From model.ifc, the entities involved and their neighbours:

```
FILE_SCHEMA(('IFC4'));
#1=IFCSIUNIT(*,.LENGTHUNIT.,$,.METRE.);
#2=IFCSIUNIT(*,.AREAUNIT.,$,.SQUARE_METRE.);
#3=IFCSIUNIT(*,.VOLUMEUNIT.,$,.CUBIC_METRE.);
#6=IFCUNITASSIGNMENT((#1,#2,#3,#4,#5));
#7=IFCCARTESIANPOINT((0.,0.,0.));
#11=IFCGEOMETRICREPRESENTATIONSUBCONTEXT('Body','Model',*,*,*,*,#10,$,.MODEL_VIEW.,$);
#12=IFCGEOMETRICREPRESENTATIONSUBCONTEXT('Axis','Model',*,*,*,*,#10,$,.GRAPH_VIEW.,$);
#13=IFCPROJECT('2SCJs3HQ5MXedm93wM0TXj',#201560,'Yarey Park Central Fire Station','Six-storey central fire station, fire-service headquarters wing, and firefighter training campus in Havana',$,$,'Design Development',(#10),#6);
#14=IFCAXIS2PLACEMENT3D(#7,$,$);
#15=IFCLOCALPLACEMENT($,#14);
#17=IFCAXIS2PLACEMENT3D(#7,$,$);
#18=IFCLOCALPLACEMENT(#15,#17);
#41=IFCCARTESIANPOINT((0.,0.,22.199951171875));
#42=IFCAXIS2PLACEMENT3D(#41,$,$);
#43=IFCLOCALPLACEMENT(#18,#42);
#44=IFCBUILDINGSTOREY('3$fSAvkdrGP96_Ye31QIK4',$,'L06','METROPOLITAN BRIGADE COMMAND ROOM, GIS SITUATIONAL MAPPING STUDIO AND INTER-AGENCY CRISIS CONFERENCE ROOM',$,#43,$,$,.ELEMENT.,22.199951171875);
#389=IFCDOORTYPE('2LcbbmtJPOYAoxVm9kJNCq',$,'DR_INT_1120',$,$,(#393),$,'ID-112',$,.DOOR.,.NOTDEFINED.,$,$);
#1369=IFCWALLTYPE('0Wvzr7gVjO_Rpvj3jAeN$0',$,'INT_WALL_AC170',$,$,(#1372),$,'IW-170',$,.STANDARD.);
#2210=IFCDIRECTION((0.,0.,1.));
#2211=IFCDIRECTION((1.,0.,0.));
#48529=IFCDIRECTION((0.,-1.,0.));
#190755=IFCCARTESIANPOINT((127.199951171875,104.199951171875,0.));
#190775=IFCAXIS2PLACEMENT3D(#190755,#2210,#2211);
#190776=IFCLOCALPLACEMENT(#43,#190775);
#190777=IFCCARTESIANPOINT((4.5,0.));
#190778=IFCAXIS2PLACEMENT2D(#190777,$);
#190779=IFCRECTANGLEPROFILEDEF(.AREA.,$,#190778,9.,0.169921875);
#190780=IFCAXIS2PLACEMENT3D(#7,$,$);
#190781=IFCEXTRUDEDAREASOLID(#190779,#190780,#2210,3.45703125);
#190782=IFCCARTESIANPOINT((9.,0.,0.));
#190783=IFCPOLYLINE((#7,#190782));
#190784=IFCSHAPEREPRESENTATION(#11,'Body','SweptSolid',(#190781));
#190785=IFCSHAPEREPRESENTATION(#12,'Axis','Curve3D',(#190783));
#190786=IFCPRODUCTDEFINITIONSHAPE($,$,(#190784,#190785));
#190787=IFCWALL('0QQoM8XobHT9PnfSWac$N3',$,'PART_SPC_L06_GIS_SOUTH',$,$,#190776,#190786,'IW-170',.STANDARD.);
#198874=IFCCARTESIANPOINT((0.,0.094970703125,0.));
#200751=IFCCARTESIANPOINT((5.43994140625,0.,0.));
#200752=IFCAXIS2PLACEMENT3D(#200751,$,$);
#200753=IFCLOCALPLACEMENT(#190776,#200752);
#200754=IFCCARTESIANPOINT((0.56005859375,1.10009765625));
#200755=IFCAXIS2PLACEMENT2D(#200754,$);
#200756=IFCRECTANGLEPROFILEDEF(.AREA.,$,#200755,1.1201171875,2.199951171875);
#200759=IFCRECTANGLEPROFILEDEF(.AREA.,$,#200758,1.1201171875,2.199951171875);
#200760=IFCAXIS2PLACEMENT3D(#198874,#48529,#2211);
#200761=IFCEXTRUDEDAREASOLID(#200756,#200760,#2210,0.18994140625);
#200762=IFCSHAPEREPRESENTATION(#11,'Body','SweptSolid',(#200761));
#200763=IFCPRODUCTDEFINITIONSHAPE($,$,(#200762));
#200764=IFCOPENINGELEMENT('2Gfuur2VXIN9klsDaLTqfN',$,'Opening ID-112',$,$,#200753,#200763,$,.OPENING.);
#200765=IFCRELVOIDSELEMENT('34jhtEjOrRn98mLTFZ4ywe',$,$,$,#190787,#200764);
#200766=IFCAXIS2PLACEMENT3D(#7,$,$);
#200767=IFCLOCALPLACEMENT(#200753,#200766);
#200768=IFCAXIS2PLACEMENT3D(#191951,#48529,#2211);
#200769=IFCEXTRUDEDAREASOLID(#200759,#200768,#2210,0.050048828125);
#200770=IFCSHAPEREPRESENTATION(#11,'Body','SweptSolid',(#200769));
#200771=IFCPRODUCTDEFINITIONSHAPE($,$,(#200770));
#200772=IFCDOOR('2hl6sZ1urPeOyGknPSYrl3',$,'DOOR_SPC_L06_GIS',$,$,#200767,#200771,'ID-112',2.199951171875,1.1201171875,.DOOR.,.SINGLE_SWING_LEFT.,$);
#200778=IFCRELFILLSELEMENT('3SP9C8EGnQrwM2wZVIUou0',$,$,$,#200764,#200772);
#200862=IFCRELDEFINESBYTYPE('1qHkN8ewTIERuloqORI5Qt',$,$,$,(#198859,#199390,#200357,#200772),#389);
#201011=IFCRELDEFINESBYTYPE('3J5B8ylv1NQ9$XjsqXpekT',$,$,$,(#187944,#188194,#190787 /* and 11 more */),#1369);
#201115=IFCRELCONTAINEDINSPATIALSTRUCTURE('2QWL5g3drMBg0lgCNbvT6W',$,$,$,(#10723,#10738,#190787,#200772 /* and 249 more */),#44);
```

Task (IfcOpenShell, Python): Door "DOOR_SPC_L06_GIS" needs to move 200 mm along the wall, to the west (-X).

```python
import ifcopenshell
import ifcopenshell.api.geometry
import ifcopenshell.util.placement
import ifcopenshell.util.unit

model = ifcopenshell.open("model.ifc")
unit_scale = ifcopenshell.util.unit.calculate_unit_scale(model)

door = model.by_guid("2hl6sZ1urPeOyGknPSYrl3")
opening = door.FillsVoids[0].RelatingOpeningElement
wall = opening.VoidsElements[0].RelatingBuildingElement

wall_matrix = ifcopenshell.util.placement.get_local_placement(wall.ObjectPlacement)
shift = wall_matrix[:3, 0] * -0.2 / unit_scale
before = ifcopenshell.util.placement.get_local_placement(door.ObjectPlacement)[:3, 3].copy()

# The door is placed relative to its opening, so it follows when the opening moves.
matrix = ifcopenshell.util.placement.get_local_placement(opening.ObjectPlacement)
matrix[:3, 3] += shift
ifcopenshell.api.geometry.edit_object_placement(
    model, product=opening, matrix=matrix, is_si=False, should_transform_children=True
)

after = ifcopenshell.util.placement.get_local_placement(door.ObjectPlacement)[:3, 3]
print("door moved by", (after - before).round(3) + 0.0)

model.write("model-out.ifc")
```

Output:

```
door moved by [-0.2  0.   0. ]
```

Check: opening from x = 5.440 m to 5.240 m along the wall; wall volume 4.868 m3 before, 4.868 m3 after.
